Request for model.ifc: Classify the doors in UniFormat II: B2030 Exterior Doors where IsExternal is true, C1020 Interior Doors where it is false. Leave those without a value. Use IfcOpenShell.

First a look at what the model holds.

```python
import ifcopenshell
import ifcopenshell.util.element

model = ifcopenshell.open("model.ifc")
print(model.schema)
print("classifications:", [c.Name for c in model.by_type("IfcClassification")])
values = [ifcopenshell.util.element.get_pset(e, "Pset_DoorCommon", "IsExternal") for e in model.by_type("IfcDoor")]
for value in (True, False, None):
    print("IsExternal", value, values.count(value))
```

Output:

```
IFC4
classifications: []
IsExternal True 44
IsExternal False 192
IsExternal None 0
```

```python
import ifcopenshell
import ifcopenshell.api.classification
import ifcopenshell.util.element

model = ifcopenshell.open("model.ifc")

system = ifcopenshell.api.classification.add_classification(model, classification="UniFormat II")

doors = model.by_type("IfcDoor")
external = {e: ifcopenshell.util.element.get_pset(e, "Pset_DoorCommon", "IsExternal") for e in doors}
for flag, code, name in ((True, "B2030", "Exterior Doors"), (False, "C1020", "Interior Doors")):
    products = [e for e in doors if external[e] is flag]
    ifcopenshell.api.classification.add_reference(
        model, products=products, classification=system, identification=code, name=name
    )
    print(code, len(products))

model.write("model-out.ifc")
```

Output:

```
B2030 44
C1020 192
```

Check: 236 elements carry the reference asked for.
